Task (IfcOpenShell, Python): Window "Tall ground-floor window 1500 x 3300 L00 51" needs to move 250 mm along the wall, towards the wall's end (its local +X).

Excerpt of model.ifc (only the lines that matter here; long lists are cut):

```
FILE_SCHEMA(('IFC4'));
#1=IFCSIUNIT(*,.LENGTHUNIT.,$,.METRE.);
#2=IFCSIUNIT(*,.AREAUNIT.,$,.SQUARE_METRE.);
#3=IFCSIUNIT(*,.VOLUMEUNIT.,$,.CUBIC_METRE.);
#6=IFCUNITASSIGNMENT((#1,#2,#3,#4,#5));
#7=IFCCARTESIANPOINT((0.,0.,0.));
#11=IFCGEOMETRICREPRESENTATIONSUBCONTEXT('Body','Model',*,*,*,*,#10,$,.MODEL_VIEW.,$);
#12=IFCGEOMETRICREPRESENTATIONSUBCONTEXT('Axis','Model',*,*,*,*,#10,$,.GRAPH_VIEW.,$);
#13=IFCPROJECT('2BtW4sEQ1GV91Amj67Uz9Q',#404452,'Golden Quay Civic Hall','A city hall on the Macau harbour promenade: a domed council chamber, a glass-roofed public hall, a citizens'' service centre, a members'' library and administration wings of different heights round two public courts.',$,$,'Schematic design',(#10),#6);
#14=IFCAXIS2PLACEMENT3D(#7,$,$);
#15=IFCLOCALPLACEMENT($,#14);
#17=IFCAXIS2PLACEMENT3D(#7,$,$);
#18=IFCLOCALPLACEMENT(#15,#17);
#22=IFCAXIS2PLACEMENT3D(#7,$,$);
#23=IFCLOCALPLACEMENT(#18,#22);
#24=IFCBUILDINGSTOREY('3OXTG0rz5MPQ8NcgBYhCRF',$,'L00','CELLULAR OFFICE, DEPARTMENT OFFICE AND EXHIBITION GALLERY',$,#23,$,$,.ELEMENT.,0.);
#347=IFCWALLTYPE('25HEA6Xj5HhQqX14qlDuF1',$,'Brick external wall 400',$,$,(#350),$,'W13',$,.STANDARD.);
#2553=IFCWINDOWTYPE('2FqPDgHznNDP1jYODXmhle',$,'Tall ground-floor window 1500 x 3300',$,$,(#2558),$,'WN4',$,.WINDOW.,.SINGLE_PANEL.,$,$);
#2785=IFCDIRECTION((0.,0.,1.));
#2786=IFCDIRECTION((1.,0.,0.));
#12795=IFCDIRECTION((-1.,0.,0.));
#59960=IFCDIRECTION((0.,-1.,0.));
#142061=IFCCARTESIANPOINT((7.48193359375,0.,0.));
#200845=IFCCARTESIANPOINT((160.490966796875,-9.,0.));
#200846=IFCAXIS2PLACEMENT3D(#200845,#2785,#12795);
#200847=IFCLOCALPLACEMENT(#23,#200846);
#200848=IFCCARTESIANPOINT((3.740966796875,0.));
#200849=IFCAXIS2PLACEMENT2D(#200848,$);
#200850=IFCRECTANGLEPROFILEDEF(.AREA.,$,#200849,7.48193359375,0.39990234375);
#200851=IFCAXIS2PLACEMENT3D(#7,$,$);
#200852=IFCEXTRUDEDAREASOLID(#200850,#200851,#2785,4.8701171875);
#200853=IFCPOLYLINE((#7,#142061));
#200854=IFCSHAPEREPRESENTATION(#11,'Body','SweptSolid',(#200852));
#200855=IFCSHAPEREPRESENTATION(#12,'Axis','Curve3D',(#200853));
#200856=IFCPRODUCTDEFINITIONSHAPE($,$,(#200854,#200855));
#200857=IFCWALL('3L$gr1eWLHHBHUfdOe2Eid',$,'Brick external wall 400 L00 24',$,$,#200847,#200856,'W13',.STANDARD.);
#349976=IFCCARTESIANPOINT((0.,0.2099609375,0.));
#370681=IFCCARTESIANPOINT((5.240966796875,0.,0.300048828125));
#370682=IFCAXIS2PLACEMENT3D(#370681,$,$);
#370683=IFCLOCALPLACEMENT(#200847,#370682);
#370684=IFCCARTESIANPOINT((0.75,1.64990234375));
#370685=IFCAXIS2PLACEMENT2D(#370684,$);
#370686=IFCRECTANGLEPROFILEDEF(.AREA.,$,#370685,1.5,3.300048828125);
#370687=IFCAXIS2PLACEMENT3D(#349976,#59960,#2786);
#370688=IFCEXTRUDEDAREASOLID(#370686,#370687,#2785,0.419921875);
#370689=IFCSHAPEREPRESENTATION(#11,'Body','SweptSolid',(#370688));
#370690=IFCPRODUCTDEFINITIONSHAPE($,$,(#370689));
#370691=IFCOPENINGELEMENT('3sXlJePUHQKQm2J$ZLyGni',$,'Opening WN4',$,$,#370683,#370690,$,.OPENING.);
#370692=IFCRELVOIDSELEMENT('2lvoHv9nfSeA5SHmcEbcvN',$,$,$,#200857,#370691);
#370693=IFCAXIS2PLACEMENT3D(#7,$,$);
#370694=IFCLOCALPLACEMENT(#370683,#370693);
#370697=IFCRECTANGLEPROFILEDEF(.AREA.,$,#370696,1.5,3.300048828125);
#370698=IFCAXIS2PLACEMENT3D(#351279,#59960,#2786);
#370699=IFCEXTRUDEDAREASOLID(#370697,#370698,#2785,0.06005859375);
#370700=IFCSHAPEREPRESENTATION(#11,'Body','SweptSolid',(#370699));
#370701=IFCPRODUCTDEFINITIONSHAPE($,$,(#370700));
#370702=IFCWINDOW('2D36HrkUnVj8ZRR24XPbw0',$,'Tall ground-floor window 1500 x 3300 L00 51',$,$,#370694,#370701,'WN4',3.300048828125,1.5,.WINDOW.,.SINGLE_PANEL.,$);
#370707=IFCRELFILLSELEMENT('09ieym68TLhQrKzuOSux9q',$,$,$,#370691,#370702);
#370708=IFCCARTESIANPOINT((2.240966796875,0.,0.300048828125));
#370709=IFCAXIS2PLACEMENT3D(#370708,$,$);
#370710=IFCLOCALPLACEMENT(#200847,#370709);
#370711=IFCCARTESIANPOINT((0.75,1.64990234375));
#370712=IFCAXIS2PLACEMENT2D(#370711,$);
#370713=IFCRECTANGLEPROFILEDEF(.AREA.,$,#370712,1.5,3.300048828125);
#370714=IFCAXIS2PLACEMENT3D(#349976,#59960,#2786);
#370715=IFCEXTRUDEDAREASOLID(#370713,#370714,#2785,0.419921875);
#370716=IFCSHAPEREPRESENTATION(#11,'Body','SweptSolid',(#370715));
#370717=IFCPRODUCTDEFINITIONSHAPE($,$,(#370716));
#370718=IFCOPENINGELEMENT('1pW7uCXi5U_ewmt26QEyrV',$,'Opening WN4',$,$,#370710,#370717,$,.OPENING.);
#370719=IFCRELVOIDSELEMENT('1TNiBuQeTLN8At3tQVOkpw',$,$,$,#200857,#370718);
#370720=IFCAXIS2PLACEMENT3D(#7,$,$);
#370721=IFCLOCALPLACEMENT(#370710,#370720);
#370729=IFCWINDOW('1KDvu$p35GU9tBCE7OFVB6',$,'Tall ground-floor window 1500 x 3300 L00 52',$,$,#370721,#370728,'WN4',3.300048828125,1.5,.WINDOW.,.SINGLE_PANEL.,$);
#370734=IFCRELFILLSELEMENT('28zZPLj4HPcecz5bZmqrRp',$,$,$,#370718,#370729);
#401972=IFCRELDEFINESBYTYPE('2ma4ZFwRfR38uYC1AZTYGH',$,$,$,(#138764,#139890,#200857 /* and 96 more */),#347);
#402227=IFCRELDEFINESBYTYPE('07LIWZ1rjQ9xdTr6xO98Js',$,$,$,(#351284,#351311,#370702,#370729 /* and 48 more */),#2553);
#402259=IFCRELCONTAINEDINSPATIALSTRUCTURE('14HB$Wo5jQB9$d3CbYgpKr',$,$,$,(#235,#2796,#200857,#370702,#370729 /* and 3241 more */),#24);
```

```python
import ifcopenshell
import ifcopenshell.api.geometry
import ifcopenshell.util.placement
import ifcopenshell.util.unit

model = ifcopenshell.open("model.ifc")
unit_scale = ifcopenshell.util.unit.calculate_unit_scale(model)

window = model.by_guid("2D36HrkUnVj8ZRR24XPbw0")
opening = window.FillsVoids[0].RelatingOpeningElement
wall = opening.VoidsElements[0].RelatingBuildingElement

wall_matrix = ifcopenshell.util.placement.get_local_placement(wall.ObjectPlacement)
shift = wall_matrix[:3, 0] * 0.25 / unit_scale
before = ifcopenshell.util.placement.get_local_placement(window.ObjectPlacement)[:3, 3].copy()

# The window is placed relative to its opening, so it follows when the opening moves.
matrix = ifcopenshell.util.placement.get_local_placement(opening.ObjectPlacement)
matrix[:3, 3] += shift
ifcopenshell.api.geometry.edit_object_placement(
    model, product=opening, matrix=matrix, is_si=False, should_transform_children=True
)

after = ifcopenshell.util.placement.get_local_placement(window.ObjectPlacement)[:3, 3]
print("window moved by", (after - before).round(3) + 0.0)

model.write("model_rev.ifc")
```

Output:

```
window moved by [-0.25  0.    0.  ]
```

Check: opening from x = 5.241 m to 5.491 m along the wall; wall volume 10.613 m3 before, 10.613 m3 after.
